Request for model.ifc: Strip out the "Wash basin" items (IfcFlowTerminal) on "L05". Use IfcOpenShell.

First a look at what the model holds.

```python
import ifcopenshell
import ifcopenshell.util.element

model = ifcopenshell.open("model.ifc")
print(model.schema)
storey = next(s for s in model.by_type("IfcBuildingStorey") if s.Name == "L05")
terminals = [e for e in ifcopenshell.util.element.get_decomposition(storey) if e.is_a("IfcFlowTerminal")]
seen = {}
for e in terminals:
    element_type = ifcopenshell.util.element.get_type(e)
    name = element_type.Name if element_type not in (None, e) else None
    seen[name] = seen.get(name, 0) + 1
for name, count in sorted(seen.items(), key=str):
    print(count, "x", name)
```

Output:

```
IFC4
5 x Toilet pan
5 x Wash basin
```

```python
import ifcopenshell
import ifcopenshell.api.root
import ifcopenshell.util.element

model = ifcopenshell.open("model.ifc")

storey = next(s for s in model.by_type("IfcBuildingStorey") if s.Name == "L05")
terminals = [e for e in ifcopenshell.util.element.get_decomposition(storey) if e.is_a("IfcFlowTerminal")]
targets = [e for e in terminals if (t := ifcopenshell.util.element.get_type(e)) not in (None, e) and t.Name == "Wash basin"]

for e in targets:
    ifcopenshell.api.root.remove_product(model, product=e)
print(len(targets), "removed")

model.write("model_rev.ifc")
```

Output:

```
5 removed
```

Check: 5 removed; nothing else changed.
